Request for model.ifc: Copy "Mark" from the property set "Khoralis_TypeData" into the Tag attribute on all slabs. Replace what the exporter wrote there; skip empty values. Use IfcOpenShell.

First a look at what the model holds.

```python
import ifcopenshell
import ifcopenshell.util.element

model = ifcopenshell.open("model.ifc")
print(model.schema)
slabs = model.by_type("IfcSlab")
print(len(slabs), "slabs")
for e in slabs[:8]:
    source = ifcopenshell.util.element.get_pset(e, "Khoralis_TypeData", "Mark")
    target = e.Tag
    print(e.id(), repr(source), repr(target), sep=" | ")
```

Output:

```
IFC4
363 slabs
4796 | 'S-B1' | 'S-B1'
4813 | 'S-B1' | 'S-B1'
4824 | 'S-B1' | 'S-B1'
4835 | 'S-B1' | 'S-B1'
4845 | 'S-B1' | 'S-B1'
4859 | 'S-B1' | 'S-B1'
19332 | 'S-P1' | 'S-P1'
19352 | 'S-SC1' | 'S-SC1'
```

```python
import ifcopenshell
import ifcopenshell.util.element

model = ifcopenshell.open("model.ifc")

count = 0
for e in model.by_type("IfcSlab"):
    value = ifcopenshell.util.element.get_pset(e, "Khoralis_TypeData", "Mark")
    current = e.Tag
    if not value or not value.strip() or current == value:
        continue
    e.Tag = value
    count += 1

print(count, "slabs updated")

model.write("model_v2.ifc")
```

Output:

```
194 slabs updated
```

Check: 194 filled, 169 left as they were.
